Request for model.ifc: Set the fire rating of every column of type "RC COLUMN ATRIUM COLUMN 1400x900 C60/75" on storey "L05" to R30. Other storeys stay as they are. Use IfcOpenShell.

First a look at what the model holds.

```python
import ifcopenshell
import ifcopenshell.util.element

model = ifcopenshell.open("model.ifc")
print(model.schema)
storey = next(s for s in model.by_type("IfcBuildingStorey") if s.Name == "L05")
columns = [e for e in ifcopenshell.util.element.get_decomposition(storey) if e.is_a("IfcColumn")]
seen = {}
for e in columns:
    element_type = ifcopenshell.util.element.get_type(e)
    key = (element_type.Name if element_type != e and element_type else None, ifcopenshell.util.element.get_pset(e, "Pset_ColumnCommon", "FireRating"))
    seen[key] = seen.get(key, 0) + 1
for (name, value), count in sorted(seen.items(), key=str):
    print(count, "x", name, "|", value)
```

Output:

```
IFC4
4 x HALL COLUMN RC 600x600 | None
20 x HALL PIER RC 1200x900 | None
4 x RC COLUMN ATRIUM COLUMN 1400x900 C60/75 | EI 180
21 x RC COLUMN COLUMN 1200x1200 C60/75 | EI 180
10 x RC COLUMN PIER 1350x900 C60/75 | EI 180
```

```python
import ifcopenshell
import ifcopenshell.api.pset
import ifcopenshell.util.element

model = ifcopenshell.open("model.ifc")

storey = next(s for s in model.by_type("IfcBuildingStorey") if s.Name == "L05")
columns = [e for e in ifcopenshell.util.element.get_decomposition(storey) if e.is_a("IfcColumn")]

count = 0
for e in columns:
    element_type = ifcopenshell.util.element.get_type(e)
    if element_type in (None, e) or element_type.Name != "RC COLUMN ATRIUM COLUMN 1400x900 C60/75":
        continue
    found = ifcopenshell.util.element.get_pset(e, "Pset_ColumnCommon", should_inherit=False)
    if found:
        pset = model.by_id(found["id"])
        if len(ifcopenshell.util.element.get_elements_by_pset(pset)) > 1:
            pset = ifcopenshell.api.pset.unshare_pset(model, products=[e], pset=pset)[0]
    else:
        pset = ifcopenshell.api.pset.add_pset(model, product=e, name="Pset_ColumnCommon")
    ifcopenshell.api.pset.edit_pset(model, pset=pset, properties={"FireRating": "R30"})
    count += 1

print(count, "columns updated")

model.write("model_updated.ifc")
```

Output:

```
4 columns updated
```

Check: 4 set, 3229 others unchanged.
